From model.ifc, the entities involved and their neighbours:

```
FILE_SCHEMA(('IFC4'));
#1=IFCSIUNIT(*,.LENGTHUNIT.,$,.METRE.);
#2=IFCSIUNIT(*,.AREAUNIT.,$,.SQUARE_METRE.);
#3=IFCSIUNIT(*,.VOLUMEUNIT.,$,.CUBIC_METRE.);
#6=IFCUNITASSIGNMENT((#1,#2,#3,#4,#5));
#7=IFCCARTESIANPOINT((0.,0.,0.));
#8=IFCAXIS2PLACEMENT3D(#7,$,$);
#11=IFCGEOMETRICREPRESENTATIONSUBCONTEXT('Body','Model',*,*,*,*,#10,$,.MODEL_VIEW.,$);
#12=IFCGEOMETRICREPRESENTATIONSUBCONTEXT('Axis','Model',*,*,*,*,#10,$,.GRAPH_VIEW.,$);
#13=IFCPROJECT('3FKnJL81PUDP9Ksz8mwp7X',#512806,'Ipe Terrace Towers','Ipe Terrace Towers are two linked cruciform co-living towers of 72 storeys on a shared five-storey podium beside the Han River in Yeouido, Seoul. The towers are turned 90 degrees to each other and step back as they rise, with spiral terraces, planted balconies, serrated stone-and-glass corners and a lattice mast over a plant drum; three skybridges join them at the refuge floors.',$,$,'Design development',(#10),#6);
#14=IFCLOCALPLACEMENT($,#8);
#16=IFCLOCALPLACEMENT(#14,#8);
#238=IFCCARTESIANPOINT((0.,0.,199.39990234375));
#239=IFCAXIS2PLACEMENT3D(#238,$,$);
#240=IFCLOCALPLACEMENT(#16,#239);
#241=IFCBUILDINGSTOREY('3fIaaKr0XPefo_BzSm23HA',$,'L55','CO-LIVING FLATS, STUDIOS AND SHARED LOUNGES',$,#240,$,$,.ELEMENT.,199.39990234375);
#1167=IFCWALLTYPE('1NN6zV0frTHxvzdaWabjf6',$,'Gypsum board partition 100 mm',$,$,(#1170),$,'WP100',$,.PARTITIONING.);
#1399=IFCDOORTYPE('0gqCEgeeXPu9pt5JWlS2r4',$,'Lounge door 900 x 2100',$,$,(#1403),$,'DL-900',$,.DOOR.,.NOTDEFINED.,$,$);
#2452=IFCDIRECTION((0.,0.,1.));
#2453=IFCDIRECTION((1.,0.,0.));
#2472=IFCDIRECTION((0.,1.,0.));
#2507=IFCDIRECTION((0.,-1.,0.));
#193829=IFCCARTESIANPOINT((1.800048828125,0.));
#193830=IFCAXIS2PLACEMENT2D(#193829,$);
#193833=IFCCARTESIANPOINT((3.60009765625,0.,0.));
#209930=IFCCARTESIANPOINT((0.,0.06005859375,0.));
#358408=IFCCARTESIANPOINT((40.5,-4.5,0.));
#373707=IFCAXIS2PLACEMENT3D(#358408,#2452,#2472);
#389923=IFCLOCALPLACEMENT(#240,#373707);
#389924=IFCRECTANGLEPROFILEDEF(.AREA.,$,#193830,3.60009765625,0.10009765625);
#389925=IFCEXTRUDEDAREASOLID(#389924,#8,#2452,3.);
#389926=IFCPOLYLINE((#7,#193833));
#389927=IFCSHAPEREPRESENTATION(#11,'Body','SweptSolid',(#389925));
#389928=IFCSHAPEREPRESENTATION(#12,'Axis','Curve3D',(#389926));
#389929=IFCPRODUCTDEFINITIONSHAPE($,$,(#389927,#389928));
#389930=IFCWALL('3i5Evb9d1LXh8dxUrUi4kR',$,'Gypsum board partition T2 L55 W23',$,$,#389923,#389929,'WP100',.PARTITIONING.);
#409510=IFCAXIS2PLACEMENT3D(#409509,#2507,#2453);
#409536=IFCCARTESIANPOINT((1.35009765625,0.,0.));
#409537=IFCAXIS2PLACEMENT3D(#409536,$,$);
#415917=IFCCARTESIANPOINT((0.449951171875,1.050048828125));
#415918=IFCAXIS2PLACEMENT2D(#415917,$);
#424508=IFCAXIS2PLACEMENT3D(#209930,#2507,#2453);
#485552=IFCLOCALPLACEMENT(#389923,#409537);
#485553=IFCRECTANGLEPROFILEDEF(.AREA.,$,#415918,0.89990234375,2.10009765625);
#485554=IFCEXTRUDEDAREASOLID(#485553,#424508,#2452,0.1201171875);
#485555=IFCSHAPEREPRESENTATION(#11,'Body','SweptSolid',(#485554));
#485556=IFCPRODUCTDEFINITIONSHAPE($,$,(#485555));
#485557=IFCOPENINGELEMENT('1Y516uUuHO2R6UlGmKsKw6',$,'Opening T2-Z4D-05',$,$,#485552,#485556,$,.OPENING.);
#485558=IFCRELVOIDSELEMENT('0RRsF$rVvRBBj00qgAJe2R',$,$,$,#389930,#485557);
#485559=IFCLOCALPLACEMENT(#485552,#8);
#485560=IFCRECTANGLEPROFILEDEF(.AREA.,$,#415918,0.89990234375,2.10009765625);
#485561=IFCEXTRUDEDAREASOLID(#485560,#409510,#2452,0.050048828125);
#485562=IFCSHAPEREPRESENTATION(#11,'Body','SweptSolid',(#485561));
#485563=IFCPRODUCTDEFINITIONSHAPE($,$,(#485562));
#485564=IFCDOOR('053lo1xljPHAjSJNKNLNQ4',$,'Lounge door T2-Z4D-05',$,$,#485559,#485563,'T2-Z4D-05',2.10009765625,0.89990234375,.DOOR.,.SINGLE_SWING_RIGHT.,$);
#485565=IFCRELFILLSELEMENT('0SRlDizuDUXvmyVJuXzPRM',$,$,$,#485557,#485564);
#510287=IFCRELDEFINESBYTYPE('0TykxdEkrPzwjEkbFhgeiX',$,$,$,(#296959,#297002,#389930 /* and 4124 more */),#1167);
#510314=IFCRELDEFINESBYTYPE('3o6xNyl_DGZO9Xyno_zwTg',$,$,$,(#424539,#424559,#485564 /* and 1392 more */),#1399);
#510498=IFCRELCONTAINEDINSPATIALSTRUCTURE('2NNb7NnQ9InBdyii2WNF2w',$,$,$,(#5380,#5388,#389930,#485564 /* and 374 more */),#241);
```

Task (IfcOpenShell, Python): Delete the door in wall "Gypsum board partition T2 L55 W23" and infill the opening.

```python
import ifcopenshell
import ifcopenshell.api.feature
import ifcopenshell.api.root
import ifcopenshell.geom
import ifcopenshell.util.shape

model = ifcopenshell.open("model.ifc")
settings = ifcopenshell.geom.settings()


def volume(element):
    """Net volume in cubic metres, openings subtracted."""
    shape = ifcopenshell.geom.create_shape(settings, element)
    return ifcopenshell.util.shape.get_volume(shape.geometry)


door = model.by_id(485564)
opening = door.FillsVoids[0].RelatingOpeningElement
wall = opening.VoidsElements[0].RelatingBuildingElement
before = volume(wall)

ifcopenshell.api.root.remove_product(model, product=door)
ifcopenshell.api.feature.remove_feature(model, feature=opening)

after = volume(wall)

print(f"wall volume {before:.3f} -> {after:.3f} m3")

model.write("model_updated.ifc")
```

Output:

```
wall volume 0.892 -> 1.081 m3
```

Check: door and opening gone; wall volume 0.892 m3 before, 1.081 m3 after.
